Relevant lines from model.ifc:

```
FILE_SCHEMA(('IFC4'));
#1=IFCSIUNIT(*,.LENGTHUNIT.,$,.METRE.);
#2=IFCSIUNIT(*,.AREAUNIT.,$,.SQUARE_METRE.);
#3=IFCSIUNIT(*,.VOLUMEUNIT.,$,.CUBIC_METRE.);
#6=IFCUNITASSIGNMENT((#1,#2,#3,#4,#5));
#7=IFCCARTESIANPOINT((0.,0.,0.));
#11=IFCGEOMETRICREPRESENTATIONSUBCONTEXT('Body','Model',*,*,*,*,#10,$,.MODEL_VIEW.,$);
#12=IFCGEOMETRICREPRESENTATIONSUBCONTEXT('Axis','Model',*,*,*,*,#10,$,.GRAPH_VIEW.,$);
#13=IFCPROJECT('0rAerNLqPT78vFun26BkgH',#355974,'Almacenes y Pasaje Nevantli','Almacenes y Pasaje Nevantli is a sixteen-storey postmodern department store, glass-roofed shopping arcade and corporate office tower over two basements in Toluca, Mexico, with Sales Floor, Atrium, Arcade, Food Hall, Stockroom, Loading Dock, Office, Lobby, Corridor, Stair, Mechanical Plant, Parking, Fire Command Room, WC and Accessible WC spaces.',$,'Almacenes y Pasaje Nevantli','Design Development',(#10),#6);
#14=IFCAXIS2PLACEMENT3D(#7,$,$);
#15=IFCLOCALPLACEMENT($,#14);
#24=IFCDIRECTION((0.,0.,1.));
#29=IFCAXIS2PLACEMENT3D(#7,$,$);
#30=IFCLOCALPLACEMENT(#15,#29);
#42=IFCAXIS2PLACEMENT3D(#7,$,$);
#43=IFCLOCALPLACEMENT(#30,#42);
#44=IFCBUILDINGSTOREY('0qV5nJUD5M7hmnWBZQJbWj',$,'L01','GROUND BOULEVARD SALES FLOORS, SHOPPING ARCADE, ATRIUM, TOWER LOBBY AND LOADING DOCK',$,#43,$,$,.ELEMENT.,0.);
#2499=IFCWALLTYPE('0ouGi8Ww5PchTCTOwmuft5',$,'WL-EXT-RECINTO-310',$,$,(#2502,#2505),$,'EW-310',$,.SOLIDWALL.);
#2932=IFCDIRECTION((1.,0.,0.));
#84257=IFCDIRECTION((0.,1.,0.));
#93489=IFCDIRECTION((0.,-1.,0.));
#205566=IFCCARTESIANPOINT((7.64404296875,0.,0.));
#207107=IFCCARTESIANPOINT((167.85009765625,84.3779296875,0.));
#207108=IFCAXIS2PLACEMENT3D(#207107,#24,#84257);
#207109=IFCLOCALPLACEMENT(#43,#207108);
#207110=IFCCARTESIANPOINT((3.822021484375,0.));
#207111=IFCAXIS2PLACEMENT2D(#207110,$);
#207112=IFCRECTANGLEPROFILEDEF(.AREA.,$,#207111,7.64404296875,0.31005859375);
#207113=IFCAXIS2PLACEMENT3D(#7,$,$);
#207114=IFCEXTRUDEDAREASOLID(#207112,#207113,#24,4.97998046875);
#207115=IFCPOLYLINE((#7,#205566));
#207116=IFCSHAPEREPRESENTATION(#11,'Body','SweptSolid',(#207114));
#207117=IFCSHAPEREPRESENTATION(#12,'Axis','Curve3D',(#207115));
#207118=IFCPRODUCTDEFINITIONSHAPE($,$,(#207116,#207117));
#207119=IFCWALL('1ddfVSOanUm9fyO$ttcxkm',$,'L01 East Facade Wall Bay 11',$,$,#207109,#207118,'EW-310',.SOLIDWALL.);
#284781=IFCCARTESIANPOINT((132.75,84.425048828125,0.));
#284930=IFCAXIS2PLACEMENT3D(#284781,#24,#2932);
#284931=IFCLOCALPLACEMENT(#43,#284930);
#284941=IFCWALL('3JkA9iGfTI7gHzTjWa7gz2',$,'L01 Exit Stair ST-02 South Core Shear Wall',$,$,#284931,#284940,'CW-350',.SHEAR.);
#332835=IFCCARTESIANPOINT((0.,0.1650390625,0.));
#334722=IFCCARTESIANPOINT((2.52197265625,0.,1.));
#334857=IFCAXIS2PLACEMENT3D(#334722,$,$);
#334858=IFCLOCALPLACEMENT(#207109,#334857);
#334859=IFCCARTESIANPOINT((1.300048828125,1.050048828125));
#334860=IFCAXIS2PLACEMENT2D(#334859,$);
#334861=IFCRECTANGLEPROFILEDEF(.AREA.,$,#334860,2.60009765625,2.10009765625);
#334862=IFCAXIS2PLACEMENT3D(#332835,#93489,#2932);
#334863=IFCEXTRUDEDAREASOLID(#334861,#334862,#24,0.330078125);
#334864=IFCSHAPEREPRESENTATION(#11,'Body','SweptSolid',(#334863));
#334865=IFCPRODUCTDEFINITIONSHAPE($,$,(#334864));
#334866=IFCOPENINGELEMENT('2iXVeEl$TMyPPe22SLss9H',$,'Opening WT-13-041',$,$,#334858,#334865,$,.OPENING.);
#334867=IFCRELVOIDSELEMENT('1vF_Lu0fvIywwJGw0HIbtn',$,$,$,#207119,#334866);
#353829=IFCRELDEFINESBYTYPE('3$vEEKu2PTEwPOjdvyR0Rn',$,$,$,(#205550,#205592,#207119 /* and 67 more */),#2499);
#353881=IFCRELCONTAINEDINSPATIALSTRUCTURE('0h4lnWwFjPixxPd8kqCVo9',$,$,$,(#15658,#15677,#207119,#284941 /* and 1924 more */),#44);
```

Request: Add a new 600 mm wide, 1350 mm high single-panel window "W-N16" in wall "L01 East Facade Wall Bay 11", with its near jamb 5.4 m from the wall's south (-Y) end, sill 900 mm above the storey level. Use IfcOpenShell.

```python
import numpy as np
import ifcopenshell
import ifcopenshell.api.feature
import ifcopenshell.api.geometry
import ifcopenshell.api.root
import ifcopenshell.api.spatial
import ifcopenshell.geom
import ifcopenshell.util.element
import ifcopenshell.util.placement
import ifcopenshell.util.representation
import ifcopenshell.util.shape
import ifcopenshell.util.unit

model = ifcopenshell.open("model.ifc")
unit_scale = ifcopenshell.util.unit.calculate_unit_scale(model)
settings = ifcopenshell.geom.settings()


def volume(element):
    """Net volume in cubic metres, openings subtracted."""
    shape = ifcopenshell.geom.create_shape(settings, element)
    return ifcopenshell.util.shape.get_volume(shape.geometry)


wall = model.by_guid("1ddfVSOanUm9fyO$ttcxkm")
storey = ifcopenshell.util.element.get_container(wall, ifc_class="IfcBuildingStorey")
context = ifcopenshell.util.representation.get_context(model, "Model", "Body", "MODEL_VIEW")
before = volume(wall)

width, height, from_end, sill = 0.6, 1.35, 5.4, 0.9  # metres

# The wall runs along its own X axis, and the end named is its -X end.
wall_shape = ifcopenshell.geom.create_shape(settings, wall)
x, y, z = ifcopenshell.util.shape.get_vertices(wall_shape.geometry).T
start = x.min() + from_end
face, thickness = float(y.min()), float(y.max() - y.min())
wall_matrix = ifcopenshell.util.placement.get_local_placement(wall.ObjectPlacement)
level = ifcopenshell.util.placement.get_local_placement(storey.ObjectPlacement)[2, 3]


def in_wall(x, y):
    """Placement at x, y metres in the wall's axes, at sill height."""
    matrix = wall_matrix.copy()
    matrix[:, 3] = wall_matrix @ np.array([x / unit_scale, y / unit_scale, 0.0, 1.0])
    matrix[2, 3] = level + sill / unit_scale
    return matrix


# Opening: a box that overshoots both wall faces by 50 mm.
opening = ifcopenshell.api.root.create_entity(model, ifc_class="IfcOpeningElement", predefined_type="OPENING")
box = ifcopenshell.api.geometry.add_wall_representation(
    model, context=context, length=width, height=height, thickness=thickness + 0.1
)
ifcopenshell.api.geometry.assign_representation(model, product=opening, representation=box)
ifcopenshell.api.geometry.edit_object_placement(model, product=opening, matrix=in_wall(start, face - 0.05), is_si=False)
ifcopenshell.api.feature.add_feature(model, feature=opening, element=wall)

window = ifcopenshell.api.root.create_entity(model, ifc_class="IfcWindow", name="W-N16", predefined_type="WINDOW")
window.OverallWidth, window.OverallHeight = width / unit_scale, height / unit_scale
window.PartitioningType = "SINGLE_PANEL"
body = ifcopenshell.api.geometry.add_window_representation(
    model,
    context=context,
    overall_width=window.OverallWidth,
    overall_height=window.OverallHeight,
    partition_type="SINGLE_PANEL",
)
ifcopenshell.api.geometry.assign_representation(model, product=window, representation=body)
ifcopenshell.api.spatial.assign_container(model, products=[window], relating_structure=storey)
ifcopenshell.api.feature.add_filling(model, opening=opening, element=window)

# Centre the window in the wall's thickness.
ifcopenshell.api.geometry.edit_object_placement(model, product=window, matrix=in_wall(start, face), is_si=False)
window_shape = ifcopenshell.geom.create_shape(settings, window)
depth = ifcopenshell.util.shape.get_vertices(window_shape.geometry)[:, 1]
offset = face + thickness / 2 - (depth.min() + depth.max()) / 2
ifcopenshell.api.geometry.edit_object_placement(model, product=window, matrix=in_wall(start, offset), is_si=False)

after = volume(wall)

print(f"wall volume {before:.3f} -> {after:.3f} m3")

model.write("model_updated.ifc")
```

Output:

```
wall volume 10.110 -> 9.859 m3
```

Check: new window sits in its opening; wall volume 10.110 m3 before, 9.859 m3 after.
